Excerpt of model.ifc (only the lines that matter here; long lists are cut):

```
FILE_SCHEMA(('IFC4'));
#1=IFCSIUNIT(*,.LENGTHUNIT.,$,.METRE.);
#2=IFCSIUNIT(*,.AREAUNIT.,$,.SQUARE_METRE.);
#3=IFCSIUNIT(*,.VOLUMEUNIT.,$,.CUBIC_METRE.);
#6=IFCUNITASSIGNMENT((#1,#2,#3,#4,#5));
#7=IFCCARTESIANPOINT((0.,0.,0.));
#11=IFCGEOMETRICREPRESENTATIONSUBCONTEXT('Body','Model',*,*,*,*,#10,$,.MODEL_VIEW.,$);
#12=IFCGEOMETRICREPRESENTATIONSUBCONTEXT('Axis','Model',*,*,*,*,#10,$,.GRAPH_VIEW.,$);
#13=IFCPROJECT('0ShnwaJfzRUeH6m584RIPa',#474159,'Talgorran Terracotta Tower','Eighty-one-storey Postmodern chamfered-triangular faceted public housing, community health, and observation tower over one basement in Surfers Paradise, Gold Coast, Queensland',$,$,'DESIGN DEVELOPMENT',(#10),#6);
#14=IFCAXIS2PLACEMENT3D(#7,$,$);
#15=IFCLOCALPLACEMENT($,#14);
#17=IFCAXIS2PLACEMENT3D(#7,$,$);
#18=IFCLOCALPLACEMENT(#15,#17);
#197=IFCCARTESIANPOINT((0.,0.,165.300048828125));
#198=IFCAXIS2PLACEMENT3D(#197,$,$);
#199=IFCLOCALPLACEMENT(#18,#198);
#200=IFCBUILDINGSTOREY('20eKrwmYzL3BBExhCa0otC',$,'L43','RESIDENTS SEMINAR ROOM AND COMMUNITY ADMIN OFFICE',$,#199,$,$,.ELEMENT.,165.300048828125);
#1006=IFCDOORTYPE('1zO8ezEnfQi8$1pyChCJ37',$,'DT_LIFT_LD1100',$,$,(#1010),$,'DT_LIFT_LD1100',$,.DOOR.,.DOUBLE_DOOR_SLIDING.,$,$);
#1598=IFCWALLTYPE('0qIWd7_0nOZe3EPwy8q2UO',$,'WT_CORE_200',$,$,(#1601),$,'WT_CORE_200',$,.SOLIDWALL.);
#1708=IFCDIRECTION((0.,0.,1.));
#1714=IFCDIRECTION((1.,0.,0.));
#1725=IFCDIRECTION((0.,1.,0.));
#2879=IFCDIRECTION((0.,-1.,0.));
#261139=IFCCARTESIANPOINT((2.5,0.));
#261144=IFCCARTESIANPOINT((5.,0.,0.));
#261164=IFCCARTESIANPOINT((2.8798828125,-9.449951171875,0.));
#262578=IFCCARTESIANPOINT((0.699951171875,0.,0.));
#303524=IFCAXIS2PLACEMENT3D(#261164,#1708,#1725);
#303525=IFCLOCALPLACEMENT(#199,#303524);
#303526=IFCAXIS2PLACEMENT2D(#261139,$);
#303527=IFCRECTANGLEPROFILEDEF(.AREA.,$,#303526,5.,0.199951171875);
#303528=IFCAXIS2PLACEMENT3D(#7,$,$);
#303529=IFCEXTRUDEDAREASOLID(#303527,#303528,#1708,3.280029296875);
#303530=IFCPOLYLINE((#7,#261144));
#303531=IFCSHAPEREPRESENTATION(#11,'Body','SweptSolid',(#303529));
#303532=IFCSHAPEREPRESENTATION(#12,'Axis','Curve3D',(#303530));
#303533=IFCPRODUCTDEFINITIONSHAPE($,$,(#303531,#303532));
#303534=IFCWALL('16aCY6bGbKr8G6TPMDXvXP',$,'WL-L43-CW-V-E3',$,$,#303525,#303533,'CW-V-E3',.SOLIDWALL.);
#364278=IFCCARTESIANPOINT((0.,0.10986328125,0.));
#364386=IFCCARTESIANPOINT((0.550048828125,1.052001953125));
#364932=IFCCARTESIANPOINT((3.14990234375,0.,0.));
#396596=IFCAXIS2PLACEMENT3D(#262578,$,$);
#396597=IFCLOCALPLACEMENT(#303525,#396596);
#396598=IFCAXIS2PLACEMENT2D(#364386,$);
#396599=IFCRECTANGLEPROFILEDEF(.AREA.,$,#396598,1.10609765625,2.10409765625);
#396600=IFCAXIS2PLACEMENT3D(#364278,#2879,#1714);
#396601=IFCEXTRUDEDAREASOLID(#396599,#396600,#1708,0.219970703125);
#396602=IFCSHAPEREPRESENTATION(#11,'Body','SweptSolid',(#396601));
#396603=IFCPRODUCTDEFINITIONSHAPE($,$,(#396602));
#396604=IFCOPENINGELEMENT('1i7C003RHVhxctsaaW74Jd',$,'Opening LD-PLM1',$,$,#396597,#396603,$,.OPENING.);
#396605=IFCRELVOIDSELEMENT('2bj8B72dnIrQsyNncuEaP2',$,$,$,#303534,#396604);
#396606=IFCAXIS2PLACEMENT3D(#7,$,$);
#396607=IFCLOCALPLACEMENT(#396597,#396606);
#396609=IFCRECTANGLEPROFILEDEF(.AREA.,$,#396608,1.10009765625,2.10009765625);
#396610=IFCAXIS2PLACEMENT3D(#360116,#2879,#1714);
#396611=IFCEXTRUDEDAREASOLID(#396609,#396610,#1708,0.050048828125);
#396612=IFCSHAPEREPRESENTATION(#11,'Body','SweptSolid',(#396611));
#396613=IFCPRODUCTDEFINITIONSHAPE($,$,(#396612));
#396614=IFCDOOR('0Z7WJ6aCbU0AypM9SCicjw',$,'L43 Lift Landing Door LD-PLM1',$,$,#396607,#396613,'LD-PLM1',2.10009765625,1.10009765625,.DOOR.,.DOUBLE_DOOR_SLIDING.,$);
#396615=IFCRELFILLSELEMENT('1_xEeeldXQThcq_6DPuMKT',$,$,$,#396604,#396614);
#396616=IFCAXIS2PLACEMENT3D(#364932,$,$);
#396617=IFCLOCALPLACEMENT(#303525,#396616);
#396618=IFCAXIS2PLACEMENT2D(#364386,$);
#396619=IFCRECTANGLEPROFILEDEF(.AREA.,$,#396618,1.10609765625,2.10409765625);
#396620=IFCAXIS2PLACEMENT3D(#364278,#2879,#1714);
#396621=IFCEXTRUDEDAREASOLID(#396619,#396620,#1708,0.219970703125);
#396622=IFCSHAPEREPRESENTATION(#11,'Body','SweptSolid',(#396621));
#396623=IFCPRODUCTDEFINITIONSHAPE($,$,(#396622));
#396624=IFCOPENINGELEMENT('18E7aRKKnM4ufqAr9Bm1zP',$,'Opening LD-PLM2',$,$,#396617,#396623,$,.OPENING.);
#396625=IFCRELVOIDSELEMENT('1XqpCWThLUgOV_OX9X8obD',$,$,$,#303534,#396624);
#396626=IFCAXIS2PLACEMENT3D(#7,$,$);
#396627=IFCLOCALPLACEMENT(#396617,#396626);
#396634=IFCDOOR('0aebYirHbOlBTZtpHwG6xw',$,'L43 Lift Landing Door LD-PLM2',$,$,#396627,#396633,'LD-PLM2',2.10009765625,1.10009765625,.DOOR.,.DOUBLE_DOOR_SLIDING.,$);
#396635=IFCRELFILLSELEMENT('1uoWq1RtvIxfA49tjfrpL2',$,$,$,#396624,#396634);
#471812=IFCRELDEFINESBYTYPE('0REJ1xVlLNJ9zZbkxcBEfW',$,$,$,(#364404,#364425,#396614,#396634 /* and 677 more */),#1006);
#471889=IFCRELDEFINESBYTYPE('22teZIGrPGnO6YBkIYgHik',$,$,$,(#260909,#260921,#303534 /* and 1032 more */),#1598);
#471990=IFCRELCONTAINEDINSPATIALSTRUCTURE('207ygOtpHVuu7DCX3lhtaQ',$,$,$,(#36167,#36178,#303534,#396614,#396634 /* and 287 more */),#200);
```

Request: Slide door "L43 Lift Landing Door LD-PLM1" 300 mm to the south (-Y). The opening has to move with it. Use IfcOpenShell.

```python
import ifcopenshell
import ifcopenshell.api.geometry
import ifcopenshell.util.placement

model = ifcopenshell.open("model.ifc")

door = model.by_guid("0Z7WJ6aCbU0AypM9SCicjw")
opening = door.FillsVoids[0].RelatingOpeningElement
wall = opening.VoidsElements[0].RelatingBuildingElement

wall_matrix = ifcopenshell.util.placement.get_local_placement(wall.ObjectPlacement)
shift = wall_matrix[:3, 0] * -0.3
before = ifcopenshell.util.placement.get_local_placement(door.ObjectPlacement)[:3, 3].copy()

# The door is placed relative to its opening, so it follows when the opening moves.
matrix = ifcopenshell.util.placement.get_local_placement(opening.ObjectPlacement)
matrix[:3, 3] += shift
ifcopenshell.api.geometry.edit_object_placement(
    model, product=opening, matrix=matrix, is_si=False, should_transform_children=True
)

after = ifcopenshell.util.placement.get_local_placement(door.ObjectPlacement)[:3, 3]
print("door moved by", (after - before).round(3) + 0.0)

model.write("model_edited.ifc")
```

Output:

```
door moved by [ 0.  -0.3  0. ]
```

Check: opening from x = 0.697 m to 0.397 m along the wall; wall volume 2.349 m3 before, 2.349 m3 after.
